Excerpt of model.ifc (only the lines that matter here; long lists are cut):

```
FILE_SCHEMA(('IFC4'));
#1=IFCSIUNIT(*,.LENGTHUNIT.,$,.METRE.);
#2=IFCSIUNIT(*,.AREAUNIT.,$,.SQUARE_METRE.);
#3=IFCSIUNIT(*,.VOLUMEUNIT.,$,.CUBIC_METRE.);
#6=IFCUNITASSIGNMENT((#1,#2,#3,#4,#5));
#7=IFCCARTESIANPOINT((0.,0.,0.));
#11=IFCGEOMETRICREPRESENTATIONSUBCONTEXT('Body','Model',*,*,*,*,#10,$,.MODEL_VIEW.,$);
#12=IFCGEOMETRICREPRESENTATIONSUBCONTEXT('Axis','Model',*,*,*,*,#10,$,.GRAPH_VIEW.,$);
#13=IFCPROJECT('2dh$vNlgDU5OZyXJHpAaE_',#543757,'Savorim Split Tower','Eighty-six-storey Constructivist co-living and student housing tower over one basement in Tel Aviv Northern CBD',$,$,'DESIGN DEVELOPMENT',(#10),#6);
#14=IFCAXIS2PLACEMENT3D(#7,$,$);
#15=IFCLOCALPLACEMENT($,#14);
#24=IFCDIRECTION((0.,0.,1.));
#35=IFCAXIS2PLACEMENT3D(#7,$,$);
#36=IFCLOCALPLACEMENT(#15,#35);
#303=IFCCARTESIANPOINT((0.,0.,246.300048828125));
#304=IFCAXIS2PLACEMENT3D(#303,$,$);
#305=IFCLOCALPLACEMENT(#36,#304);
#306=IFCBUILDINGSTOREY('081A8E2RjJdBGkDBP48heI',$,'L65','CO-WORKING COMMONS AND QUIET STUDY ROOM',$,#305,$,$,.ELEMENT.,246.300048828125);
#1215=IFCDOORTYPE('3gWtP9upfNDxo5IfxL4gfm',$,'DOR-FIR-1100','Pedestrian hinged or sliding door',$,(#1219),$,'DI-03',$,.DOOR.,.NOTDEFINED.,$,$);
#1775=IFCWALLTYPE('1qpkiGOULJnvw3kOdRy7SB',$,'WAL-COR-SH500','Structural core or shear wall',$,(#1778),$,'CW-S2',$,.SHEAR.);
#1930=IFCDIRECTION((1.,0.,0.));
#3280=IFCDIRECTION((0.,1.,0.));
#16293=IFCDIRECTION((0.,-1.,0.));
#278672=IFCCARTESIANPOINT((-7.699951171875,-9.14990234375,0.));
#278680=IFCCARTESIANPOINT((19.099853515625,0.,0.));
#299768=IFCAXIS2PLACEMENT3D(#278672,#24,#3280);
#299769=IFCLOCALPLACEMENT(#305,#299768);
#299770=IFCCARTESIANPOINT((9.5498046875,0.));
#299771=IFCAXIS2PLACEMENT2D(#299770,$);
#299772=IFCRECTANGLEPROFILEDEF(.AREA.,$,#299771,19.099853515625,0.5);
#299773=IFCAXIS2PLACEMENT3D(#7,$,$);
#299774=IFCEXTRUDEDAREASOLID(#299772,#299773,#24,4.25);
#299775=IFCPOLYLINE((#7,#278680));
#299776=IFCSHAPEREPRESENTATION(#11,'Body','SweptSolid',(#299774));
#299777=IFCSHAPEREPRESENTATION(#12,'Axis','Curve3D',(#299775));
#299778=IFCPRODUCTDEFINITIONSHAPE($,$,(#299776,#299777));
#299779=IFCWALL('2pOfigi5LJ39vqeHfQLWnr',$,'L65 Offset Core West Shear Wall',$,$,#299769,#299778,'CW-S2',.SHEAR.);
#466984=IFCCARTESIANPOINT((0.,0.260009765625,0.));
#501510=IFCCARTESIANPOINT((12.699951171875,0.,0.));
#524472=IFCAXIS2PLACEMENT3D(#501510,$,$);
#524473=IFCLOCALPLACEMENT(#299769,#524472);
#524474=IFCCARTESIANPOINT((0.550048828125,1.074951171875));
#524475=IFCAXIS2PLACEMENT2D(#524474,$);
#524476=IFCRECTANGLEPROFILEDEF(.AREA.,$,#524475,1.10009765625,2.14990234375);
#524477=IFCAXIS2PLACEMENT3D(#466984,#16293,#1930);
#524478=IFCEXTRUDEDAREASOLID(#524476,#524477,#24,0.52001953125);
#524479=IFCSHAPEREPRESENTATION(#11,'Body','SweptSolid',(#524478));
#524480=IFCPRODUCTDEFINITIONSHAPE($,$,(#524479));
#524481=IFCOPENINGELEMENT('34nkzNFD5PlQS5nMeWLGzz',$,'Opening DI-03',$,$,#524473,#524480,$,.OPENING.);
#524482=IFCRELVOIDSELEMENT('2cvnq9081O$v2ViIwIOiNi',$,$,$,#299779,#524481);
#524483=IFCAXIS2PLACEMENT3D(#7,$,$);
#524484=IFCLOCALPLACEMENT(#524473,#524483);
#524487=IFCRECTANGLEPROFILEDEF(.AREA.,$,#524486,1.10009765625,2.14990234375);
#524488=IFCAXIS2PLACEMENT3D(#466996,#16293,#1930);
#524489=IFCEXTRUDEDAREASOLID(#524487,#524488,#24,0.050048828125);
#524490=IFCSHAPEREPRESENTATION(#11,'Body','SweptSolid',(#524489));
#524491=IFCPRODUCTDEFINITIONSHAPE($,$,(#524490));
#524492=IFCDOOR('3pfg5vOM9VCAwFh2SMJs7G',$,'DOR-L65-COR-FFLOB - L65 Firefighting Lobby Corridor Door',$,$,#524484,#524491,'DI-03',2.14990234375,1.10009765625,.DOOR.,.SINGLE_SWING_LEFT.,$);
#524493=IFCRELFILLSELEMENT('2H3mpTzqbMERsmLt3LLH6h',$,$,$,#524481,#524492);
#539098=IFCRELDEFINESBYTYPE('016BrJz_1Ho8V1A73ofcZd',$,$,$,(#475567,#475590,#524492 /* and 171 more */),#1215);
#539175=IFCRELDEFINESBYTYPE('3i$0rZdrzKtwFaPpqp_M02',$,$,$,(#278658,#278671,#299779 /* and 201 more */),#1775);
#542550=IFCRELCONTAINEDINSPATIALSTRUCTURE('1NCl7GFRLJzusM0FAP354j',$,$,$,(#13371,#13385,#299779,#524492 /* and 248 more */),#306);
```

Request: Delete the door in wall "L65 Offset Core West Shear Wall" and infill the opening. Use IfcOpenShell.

```python
import ifcopenshell
import ifcopenshell.api.feature
import ifcopenshell.api.root
import ifcopenshell.geom
import ifcopenshell.util.shape

model = ifcopenshell.open("model.ifc")
settings = ifcopenshell.geom.settings()


def volume(element):
    """Net volume in cubic metres, openings subtracted."""
    shape = ifcopenshell.geom.create_shape(settings, element)
    return ifcopenshell.util.shape.get_volume(shape.geometry)


door = model.by_guid("3pfg5vOM9VCAwFh2SMJs7G")
opening = door.FillsVoids[0].RelatingOpeningElement
wall = opening.VoidsElements[0].RelatingBuildingElement
before = volume(wall)

ifcopenshell.api.root.remove_product(model, product=door)
ifcopenshell.api.feature.remove_feature(model, feature=opening)

after = volume(wall)

print(f"wall volume {before:.3f} -> {after:.3f} m3")

model.write("model_v2.ifc")
```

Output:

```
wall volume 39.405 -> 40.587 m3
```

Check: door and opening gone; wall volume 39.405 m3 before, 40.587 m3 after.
